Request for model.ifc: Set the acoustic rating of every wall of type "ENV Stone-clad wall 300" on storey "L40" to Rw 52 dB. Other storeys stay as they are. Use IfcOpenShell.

First a look at what the model holds.

```python
import ifcopenshell
import ifcopenshell.util.element

model = ifcopenshell.open("model.ifc")
print(model.schema)
storey = next(s for s in model.by_type("IfcBuildingStorey") if s.Name == "L40")
walls = [e for e in ifcopenshell.util.element.get_decomposition(storey) if e.is_a("IfcWall")]
seen = {}
for e in walls:
    element_type = ifcopenshell.util.element.get_type(e)
    key = (element_type.Name if element_type != e and element_type else None, ifcopenshell.util.element.get_pset(e, "Pset_WallCommon", "AcousticRating"))
    seen[key] = seen.get(key, 0) + 1
for (name, value), count in sorted(seen.items(), key=str):
    print(count, "x", name, "|", value)
```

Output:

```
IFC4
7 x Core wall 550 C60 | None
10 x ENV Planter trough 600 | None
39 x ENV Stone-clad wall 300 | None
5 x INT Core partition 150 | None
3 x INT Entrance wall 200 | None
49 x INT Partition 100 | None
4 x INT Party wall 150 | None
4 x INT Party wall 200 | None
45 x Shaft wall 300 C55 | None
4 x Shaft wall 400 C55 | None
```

```python
import ifcopenshell
import ifcopenshell.api.pset
import ifcopenshell.util.element

model = ifcopenshell.open("model.ifc")

storey = next(s for s in model.by_type("IfcBuildingStorey") if s.Name == "L40")
walls = [e for e in ifcopenshell.util.element.get_decomposition(storey) if e.is_a("IfcWall")]

count = 0
for e in walls:
    element_type = ifcopenshell.util.element.get_type(e)
    if element_type in (None, e) or element_type.Name != "ENV Stone-clad wall 300":
        continue
    found = ifcopenshell.util.element.get_pset(e, "Pset_WallCommon", should_inherit=False)
    if found:
        pset = model.by_id(found["id"])
        if len(ifcopenshell.util.element.get_elements_by_pset(pset)) > 1:
            pset = ifcopenshell.api.pset.unshare_pset(model, products=[e], pset=pset)[0]
    else:
        pset = ifcopenshell.api.pset.add_pset(model, product=e, name="Pset_WallCommon")
    ifcopenshell.api.pset.edit_pset(model, pset=pset, properties={"AcousticRating": "Rw 52 dB"})
    count += 1

print(count, "walls updated")

model.write("model-out.ifc")
```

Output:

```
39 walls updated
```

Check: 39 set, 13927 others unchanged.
